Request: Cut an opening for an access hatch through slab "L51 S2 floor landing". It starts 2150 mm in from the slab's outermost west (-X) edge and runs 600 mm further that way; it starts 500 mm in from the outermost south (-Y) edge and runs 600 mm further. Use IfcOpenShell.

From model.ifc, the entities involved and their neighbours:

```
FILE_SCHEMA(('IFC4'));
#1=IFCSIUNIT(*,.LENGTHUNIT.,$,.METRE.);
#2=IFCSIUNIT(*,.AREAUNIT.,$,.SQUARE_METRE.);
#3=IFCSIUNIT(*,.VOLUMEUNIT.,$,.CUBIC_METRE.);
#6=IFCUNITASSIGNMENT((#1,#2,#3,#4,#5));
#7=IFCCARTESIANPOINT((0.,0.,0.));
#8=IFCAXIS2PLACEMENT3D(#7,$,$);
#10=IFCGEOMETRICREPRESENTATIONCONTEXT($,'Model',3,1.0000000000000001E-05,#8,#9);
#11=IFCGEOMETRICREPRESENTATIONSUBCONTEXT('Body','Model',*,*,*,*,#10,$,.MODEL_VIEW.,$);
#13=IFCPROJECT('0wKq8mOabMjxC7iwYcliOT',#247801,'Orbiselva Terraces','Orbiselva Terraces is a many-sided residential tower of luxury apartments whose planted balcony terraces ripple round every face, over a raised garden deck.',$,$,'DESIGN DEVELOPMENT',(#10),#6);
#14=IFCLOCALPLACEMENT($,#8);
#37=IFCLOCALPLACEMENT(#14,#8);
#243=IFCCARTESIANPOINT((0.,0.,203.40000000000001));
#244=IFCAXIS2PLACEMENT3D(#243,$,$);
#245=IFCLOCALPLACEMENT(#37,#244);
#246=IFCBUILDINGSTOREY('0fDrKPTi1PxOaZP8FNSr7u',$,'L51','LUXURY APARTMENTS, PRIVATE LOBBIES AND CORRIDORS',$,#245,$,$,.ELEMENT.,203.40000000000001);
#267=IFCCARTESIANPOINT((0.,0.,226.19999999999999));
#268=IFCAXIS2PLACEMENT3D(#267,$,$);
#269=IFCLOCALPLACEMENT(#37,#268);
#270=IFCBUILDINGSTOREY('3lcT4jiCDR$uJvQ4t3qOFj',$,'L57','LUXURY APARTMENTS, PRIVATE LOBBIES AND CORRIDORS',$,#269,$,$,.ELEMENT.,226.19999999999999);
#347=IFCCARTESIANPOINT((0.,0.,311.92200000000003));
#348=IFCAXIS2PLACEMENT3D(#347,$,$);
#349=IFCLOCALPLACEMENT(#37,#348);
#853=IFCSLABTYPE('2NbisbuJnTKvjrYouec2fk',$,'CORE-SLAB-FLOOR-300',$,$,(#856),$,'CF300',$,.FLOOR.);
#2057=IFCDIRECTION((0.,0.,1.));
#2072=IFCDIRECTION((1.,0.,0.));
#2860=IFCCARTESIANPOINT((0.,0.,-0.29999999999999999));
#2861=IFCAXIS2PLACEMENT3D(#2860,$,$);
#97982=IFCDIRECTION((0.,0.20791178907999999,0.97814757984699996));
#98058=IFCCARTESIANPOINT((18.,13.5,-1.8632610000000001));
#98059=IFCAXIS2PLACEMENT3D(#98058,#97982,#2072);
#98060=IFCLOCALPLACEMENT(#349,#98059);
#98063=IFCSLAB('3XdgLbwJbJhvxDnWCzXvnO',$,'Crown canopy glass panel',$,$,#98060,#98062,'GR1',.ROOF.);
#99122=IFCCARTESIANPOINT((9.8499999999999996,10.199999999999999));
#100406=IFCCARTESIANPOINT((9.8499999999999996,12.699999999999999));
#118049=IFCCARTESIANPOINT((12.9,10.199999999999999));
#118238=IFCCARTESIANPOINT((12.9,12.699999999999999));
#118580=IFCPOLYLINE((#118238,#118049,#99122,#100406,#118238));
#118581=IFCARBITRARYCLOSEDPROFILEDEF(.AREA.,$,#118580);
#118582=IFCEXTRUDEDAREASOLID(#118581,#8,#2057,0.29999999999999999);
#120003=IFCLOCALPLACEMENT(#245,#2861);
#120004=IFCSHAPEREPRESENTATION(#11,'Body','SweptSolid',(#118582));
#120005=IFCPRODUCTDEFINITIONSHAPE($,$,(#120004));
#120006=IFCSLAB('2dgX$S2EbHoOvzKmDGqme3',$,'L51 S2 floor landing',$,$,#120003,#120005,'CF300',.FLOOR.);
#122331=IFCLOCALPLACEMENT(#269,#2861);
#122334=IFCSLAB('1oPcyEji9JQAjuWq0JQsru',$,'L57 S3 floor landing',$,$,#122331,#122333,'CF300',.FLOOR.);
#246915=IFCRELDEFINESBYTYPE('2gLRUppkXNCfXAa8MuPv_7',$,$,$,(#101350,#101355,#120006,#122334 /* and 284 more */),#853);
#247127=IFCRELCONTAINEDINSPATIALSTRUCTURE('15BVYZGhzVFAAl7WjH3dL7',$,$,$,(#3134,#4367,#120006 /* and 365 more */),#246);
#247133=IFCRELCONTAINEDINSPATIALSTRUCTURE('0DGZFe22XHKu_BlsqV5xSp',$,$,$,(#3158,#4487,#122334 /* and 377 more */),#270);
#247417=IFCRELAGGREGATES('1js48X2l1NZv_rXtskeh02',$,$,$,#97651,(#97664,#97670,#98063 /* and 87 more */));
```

```python
import numpy as np
import ifcopenshell
import ifcopenshell.api.feature
import ifcopenshell.api.geometry
import ifcopenshell.api.root
import ifcopenshell.geom
import ifcopenshell.util.placement
import ifcopenshell.util.representation
import ifcopenshell.util.shape
import ifcopenshell.util.unit

model = ifcopenshell.open("model.ifc")
unit_scale = ifcopenshell.util.unit.calculate_unit_scale(model)
settings = ifcopenshell.geom.settings()


def volume(element):
    """Net volume in cubic metres, openings subtracted."""
    shape = ifcopenshell.geom.create_shape(settings, element)
    return ifcopenshell.util.shape.get_volume(shape.geometry)


slab = model.by_guid("2dgX$S2EbHoOvzKmDGqme3")
before = volume(slab)

# Extent in the slab's own axes, in metres. The edges named are its -X and -Y sides.
slab_shape = ifcopenshell.geom.create_shape(settings, slab)
vertices = ifcopenshell.util.shape.get_vertices(slab_shape.geometry)
x_min, y_min, bottom = vertices.min(axis=0)
top = vertices[:, 2].max()

opening = ifcopenshell.api.root.create_entity(model, ifc_class="IfcOpeningElement", name="Access hatch opening", predefined_type="OPENING")
context = ifcopenshell.util.representation.get_context(model, "Model", "Body", "MODEL_VIEW")
width, depth = 0.6, 0.6
outline = [(0.0, 0.0), (width, 0.0), (width, depth), (0.0, depth), (0.0, 0.0)]
# Overshoot both faces by 50 mm so the cut is clean.
shape = ifcopenshell.api.geometry.add_slab_representation(
    model, context=context, depth=top - bottom + 0.1, polyline=outline
)
ifcopenshell.api.geometry.assign_representation(model, product=opening, representation=shape)

matrix = ifcopenshell.util.placement.get_local_placement(slab.ObjectPlacement)
matrix[:, 3] = matrix @ np.append(np.array([x_min + 2.15, y_min + 0.5, bottom - 0.05]) / unit_scale, 1.0)
ifcopenshell.api.geometry.edit_object_placement(model, product=opening, matrix=matrix, is_si=False)
ifcopenshell.api.feature.add_feature(model, feature=opening, element=slab)

after = volume(slab)

print(f"slab volume {before:.3f} -> {after:.3f} m3")

model.write("model_updated.ifc")
```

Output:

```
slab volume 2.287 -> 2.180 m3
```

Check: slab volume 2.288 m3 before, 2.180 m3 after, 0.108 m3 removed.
